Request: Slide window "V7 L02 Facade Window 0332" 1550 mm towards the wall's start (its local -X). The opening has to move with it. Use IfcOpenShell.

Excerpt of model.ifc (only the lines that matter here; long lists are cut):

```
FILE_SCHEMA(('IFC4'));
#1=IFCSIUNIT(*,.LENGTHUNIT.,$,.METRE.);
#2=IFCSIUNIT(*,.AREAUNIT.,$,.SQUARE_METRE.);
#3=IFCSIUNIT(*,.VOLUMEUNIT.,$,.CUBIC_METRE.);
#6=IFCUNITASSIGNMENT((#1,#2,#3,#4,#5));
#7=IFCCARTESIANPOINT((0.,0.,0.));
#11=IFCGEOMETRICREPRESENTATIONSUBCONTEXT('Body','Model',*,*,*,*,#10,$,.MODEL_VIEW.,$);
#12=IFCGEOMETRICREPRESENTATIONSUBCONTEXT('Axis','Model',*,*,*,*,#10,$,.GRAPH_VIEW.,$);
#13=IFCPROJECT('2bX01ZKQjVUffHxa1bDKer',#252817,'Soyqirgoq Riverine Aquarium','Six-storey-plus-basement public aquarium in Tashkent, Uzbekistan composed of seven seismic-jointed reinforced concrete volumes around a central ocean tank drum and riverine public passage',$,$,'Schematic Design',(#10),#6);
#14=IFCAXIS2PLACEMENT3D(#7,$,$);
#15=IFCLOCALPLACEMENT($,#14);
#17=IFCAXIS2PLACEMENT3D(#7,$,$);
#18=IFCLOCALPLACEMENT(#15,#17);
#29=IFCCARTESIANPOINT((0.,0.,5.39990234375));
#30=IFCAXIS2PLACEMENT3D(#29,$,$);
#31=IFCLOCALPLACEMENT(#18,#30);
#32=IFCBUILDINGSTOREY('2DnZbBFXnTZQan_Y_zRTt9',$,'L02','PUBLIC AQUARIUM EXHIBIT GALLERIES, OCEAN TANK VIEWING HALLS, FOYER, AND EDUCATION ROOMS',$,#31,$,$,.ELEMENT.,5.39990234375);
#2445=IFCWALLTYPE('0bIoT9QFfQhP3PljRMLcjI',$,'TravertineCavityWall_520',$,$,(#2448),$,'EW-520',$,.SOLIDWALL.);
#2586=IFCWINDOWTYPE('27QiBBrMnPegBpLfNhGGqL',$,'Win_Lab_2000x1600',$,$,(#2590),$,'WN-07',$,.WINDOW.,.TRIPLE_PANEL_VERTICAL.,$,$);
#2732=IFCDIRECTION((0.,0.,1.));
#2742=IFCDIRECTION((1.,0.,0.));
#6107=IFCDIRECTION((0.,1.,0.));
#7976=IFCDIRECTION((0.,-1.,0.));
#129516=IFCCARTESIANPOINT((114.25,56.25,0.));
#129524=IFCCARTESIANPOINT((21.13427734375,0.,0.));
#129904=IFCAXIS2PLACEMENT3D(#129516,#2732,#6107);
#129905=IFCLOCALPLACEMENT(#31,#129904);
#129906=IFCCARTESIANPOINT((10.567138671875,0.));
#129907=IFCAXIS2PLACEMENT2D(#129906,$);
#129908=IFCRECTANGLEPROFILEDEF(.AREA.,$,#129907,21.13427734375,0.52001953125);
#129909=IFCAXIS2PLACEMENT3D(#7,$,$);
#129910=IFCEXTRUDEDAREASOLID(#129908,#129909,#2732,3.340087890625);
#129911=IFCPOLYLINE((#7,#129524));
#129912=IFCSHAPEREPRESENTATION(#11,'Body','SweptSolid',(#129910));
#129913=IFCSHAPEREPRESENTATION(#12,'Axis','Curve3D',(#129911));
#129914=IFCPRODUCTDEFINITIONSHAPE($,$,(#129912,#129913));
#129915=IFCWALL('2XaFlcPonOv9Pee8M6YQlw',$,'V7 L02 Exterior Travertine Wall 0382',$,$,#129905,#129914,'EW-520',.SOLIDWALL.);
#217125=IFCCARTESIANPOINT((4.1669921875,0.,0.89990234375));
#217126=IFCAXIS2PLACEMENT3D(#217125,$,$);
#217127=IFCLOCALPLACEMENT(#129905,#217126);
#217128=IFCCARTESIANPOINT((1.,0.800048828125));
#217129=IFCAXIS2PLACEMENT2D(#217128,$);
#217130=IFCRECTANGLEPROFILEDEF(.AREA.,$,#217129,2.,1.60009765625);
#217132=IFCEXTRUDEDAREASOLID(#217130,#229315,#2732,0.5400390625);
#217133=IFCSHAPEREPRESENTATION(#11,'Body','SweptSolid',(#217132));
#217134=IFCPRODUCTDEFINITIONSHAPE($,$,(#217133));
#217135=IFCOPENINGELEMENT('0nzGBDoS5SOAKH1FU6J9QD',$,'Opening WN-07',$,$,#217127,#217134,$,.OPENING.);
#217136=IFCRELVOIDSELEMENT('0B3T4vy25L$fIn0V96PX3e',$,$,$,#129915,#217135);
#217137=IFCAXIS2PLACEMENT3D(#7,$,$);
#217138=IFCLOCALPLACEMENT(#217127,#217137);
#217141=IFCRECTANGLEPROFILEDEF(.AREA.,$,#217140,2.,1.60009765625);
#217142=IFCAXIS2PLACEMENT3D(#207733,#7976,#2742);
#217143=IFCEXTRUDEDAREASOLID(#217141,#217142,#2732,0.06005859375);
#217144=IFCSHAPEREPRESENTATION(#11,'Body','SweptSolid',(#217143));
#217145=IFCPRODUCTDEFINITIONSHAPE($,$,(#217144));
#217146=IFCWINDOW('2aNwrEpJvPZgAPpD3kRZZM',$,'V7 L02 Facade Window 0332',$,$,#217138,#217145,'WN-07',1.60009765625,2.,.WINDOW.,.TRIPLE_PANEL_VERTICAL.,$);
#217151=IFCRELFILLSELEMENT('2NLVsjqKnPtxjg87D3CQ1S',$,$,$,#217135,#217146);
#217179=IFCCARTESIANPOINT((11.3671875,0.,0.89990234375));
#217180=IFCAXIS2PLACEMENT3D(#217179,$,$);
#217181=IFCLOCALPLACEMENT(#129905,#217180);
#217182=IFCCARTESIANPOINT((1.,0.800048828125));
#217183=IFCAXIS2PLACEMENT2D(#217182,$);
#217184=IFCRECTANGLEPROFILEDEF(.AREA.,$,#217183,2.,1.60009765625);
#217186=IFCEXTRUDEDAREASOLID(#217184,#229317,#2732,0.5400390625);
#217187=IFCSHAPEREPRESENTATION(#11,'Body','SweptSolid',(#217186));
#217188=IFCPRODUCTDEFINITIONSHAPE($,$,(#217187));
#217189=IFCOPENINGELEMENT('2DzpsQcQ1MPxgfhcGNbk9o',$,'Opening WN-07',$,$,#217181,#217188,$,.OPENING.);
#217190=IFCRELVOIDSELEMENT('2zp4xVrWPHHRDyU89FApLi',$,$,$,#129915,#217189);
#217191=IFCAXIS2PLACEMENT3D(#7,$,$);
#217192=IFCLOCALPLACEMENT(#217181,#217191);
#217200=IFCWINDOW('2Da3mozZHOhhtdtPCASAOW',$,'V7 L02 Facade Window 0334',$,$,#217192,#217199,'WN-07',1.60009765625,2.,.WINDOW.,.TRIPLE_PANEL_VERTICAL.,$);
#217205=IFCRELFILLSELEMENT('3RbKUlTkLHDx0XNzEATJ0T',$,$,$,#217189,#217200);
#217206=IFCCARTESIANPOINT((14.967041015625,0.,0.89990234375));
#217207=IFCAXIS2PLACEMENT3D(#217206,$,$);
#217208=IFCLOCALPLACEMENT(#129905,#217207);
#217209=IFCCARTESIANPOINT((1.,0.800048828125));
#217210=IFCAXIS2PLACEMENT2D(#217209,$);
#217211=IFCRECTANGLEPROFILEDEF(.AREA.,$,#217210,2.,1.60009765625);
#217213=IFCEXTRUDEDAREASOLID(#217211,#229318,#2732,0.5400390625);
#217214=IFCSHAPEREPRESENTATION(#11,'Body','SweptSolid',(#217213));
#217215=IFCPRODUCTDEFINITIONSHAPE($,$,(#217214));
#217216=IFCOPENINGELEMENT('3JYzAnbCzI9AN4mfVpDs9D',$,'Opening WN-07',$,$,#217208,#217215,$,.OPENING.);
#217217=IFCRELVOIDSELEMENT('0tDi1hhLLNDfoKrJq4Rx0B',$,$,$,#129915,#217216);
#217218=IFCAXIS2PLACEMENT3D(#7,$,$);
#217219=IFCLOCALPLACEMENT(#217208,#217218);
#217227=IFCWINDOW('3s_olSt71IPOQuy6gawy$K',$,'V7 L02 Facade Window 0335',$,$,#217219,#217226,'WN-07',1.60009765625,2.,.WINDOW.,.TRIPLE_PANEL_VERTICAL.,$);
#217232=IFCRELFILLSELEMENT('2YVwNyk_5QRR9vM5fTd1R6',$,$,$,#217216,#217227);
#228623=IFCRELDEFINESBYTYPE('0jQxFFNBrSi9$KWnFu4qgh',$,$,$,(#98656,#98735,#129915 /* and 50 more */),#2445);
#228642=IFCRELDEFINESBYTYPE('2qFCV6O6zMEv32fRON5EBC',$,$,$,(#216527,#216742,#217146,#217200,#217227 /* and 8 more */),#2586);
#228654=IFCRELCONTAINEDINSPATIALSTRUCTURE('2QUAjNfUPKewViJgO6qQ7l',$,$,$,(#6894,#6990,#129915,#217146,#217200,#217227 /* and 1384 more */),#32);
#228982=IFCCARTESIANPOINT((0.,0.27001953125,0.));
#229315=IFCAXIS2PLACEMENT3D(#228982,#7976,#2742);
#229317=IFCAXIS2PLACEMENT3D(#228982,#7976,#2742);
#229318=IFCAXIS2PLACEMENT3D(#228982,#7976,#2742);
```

```python
import ifcopenshell
import ifcopenshell.api.geometry
import ifcopenshell.util.placement

model = ifcopenshell.open("model.ifc")

window = model.by_guid("2aNwrEpJvPZgAPpD3kRZZM")
opening = window.FillsVoids[0].RelatingOpeningElement
wall = opening.VoidsElements[0].RelatingBuildingElement

wall_matrix = ifcopenshell.util.placement.get_local_placement(wall.ObjectPlacement)
shift = wall_matrix[:3, 0] * -1.55
before = ifcopenshell.util.placement.get_local_placement(window.ObjectPlacement)[:3, 3].copy()

# The window is placed relative to its opening, so it follows when the opening moves.
matrix = ifcopenshell.util.placement.get_local_placement(opening.ObjectPlacement)
matrix[:3, 3] += shift
ifcopenshell.api.geometry.edit_object_placement(
    model, product=opening, matrix=matrix, is_si=False, should_transform_children=True
)

after = ifcopenshell.util.placement.get_local_placement(window.ObjectPlacement)[:3, 3]
print("window moved by", (after - before).round(3) + 0.0)

model.write("model_v2.ifc")
```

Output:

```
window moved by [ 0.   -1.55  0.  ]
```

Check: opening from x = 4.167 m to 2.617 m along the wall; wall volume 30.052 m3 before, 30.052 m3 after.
